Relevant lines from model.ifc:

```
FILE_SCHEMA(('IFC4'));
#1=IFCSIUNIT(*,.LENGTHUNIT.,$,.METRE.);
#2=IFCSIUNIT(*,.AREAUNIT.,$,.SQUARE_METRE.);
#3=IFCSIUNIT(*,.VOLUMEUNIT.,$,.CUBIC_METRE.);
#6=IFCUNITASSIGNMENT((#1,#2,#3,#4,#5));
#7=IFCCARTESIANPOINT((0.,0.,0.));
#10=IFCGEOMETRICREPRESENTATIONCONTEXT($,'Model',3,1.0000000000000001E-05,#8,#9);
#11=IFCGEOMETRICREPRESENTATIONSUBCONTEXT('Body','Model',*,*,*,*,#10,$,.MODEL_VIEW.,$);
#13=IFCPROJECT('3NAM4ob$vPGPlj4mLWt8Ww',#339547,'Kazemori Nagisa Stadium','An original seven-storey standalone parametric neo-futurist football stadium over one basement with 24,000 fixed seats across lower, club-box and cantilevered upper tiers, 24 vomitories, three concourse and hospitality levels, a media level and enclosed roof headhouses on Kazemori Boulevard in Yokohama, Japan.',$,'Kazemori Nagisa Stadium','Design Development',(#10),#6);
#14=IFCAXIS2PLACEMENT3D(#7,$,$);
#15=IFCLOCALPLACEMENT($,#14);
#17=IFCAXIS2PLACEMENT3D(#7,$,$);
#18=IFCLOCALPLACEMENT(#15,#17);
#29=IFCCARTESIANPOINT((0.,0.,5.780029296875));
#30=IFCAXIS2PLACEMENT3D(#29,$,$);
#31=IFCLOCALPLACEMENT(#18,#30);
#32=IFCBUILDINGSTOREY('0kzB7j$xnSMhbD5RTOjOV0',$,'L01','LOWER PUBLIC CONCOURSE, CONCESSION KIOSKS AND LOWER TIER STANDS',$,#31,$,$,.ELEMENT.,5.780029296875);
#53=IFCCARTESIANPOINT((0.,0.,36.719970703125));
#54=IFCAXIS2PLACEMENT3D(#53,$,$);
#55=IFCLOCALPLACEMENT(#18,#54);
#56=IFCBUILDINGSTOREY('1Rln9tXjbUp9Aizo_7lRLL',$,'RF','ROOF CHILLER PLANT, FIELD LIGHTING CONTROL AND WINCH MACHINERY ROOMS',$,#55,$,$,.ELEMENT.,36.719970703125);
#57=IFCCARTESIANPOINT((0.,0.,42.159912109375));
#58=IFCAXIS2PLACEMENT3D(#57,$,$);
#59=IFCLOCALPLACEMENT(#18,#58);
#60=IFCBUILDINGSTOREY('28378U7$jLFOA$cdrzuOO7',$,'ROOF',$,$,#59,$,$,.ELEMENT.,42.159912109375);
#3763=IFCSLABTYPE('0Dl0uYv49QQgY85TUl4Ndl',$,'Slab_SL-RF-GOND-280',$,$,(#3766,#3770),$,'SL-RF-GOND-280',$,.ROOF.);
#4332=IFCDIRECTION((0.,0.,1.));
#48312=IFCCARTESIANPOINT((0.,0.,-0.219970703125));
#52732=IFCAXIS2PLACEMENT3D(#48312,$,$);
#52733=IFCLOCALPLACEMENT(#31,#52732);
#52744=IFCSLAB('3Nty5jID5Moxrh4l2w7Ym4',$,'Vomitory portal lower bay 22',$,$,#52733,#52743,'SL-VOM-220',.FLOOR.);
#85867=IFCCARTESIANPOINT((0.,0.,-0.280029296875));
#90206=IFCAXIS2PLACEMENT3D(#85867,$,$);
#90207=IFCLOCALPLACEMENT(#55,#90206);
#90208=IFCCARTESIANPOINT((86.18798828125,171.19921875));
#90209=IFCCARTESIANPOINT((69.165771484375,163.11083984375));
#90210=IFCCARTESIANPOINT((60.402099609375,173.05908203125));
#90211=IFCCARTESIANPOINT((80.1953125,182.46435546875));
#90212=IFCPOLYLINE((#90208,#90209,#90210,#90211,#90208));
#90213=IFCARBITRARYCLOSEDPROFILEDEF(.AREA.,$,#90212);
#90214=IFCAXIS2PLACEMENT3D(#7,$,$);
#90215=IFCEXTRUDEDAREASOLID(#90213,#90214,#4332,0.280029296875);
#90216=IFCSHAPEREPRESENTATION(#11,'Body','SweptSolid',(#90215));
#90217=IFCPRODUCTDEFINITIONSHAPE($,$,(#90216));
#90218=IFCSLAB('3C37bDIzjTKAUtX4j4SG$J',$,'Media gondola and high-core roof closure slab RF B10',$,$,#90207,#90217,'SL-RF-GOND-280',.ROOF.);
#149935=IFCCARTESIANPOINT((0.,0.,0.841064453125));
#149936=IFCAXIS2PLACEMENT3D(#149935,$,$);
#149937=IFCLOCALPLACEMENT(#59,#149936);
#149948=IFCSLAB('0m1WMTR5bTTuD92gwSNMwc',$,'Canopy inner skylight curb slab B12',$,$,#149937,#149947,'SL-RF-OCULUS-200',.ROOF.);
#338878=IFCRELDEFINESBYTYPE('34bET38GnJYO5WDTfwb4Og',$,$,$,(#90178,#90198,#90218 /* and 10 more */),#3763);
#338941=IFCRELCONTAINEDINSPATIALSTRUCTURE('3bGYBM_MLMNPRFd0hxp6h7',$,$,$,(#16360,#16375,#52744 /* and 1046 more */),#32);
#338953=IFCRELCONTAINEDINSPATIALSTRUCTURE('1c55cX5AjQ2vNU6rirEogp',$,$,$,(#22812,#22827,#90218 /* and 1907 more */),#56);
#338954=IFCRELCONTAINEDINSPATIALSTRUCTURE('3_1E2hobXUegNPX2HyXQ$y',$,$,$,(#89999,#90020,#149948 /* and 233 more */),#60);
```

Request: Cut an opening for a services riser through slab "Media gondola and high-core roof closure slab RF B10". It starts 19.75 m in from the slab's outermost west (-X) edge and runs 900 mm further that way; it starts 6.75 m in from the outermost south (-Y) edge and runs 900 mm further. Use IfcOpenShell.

```python
import numpy as np
import ifcopenshell
import ifcopenshell.api.feature
import ifcopenshell.api.geometry
import ifcopenshell.api.root
import ifcopenshell.geom
import ifcopenshell.util.placement
import ifcopenshell.util.representation
import ifcopenshell.util.shape
import ifcopenshell.util.unit

model = ifcopenshell.open("model.ifc")
unit_scale = ifcopenshell.util.unit.calculate_unit_scale(model)
settings = ifcopenshell.geom.settings()


def volume(element):
    """Net volume in cubic metres, openings subtracted."""
    shape = ifcopenshell.geom.create_shape(settings, element)
    return ifcopenshell.util.shape.get_volume(shape.geometry)


slab = model.by_guid("3C37bDIzjTKAUtX4j4SG$J")
before = volume(slab)

# Extent in the slab's own axes, in metres. The edges named are its -X and -Y sides.
slab_shape = ifcopenshell.geom.create_shape(settings, slab)
vertices = ifcopenshell.util.shape.get_vertices(slab_shape.geometry)
x_min, y_min, bottom = vertices.min(axis=0)
top = vertices[:, 2].max()

opening = ifcopenshell.api.root.create_entity(model, ifc_class="IfcOpeningElement", name="Services riser opening", predefined_type="OPENING")
context = ifcopenshell.util.representation.get_context(model, "Model", "Body", "MODEL_VIEW")
width, depth = 0.9, 0.9
outline = [(0.0, 0.0), (width, 0.0), (width, depth), (0.0, depth), (0.0, 0.0)]
# Overshoot both faces by 50 mm so the cut is clean.
shape = ifcopenshell.api.geometry.add_slab_representation(
    model, context=context, depth=top - bottom + 0.1, polyline=outline
)
ifcopenshell.api.geometry.assign_representation(model, product=opening, representation=shape)

matrix = ifcopenshell.util.placement.get_local_placement(slab.ObjectPlacement)
matrix[:, 3] = matrix @ np.append(np.array([x_min + 19.75, y_min + 6.75, bottom - 0.05]) / unit_scale, 1.0)
ifcopenshell.api.geometry.edit_object_placement(model, product=opening, matrix=matrix, is_si=False)
ifcopenshell.api.feature.add_feature(model, feature=opening, element=slab)

after = volume(slab)

print(f"slab volume {before:.3f} -> {after:.3f} m3")

model.write("model_updated.ifc")
```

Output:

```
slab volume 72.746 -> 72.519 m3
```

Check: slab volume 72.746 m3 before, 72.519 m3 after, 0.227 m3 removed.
